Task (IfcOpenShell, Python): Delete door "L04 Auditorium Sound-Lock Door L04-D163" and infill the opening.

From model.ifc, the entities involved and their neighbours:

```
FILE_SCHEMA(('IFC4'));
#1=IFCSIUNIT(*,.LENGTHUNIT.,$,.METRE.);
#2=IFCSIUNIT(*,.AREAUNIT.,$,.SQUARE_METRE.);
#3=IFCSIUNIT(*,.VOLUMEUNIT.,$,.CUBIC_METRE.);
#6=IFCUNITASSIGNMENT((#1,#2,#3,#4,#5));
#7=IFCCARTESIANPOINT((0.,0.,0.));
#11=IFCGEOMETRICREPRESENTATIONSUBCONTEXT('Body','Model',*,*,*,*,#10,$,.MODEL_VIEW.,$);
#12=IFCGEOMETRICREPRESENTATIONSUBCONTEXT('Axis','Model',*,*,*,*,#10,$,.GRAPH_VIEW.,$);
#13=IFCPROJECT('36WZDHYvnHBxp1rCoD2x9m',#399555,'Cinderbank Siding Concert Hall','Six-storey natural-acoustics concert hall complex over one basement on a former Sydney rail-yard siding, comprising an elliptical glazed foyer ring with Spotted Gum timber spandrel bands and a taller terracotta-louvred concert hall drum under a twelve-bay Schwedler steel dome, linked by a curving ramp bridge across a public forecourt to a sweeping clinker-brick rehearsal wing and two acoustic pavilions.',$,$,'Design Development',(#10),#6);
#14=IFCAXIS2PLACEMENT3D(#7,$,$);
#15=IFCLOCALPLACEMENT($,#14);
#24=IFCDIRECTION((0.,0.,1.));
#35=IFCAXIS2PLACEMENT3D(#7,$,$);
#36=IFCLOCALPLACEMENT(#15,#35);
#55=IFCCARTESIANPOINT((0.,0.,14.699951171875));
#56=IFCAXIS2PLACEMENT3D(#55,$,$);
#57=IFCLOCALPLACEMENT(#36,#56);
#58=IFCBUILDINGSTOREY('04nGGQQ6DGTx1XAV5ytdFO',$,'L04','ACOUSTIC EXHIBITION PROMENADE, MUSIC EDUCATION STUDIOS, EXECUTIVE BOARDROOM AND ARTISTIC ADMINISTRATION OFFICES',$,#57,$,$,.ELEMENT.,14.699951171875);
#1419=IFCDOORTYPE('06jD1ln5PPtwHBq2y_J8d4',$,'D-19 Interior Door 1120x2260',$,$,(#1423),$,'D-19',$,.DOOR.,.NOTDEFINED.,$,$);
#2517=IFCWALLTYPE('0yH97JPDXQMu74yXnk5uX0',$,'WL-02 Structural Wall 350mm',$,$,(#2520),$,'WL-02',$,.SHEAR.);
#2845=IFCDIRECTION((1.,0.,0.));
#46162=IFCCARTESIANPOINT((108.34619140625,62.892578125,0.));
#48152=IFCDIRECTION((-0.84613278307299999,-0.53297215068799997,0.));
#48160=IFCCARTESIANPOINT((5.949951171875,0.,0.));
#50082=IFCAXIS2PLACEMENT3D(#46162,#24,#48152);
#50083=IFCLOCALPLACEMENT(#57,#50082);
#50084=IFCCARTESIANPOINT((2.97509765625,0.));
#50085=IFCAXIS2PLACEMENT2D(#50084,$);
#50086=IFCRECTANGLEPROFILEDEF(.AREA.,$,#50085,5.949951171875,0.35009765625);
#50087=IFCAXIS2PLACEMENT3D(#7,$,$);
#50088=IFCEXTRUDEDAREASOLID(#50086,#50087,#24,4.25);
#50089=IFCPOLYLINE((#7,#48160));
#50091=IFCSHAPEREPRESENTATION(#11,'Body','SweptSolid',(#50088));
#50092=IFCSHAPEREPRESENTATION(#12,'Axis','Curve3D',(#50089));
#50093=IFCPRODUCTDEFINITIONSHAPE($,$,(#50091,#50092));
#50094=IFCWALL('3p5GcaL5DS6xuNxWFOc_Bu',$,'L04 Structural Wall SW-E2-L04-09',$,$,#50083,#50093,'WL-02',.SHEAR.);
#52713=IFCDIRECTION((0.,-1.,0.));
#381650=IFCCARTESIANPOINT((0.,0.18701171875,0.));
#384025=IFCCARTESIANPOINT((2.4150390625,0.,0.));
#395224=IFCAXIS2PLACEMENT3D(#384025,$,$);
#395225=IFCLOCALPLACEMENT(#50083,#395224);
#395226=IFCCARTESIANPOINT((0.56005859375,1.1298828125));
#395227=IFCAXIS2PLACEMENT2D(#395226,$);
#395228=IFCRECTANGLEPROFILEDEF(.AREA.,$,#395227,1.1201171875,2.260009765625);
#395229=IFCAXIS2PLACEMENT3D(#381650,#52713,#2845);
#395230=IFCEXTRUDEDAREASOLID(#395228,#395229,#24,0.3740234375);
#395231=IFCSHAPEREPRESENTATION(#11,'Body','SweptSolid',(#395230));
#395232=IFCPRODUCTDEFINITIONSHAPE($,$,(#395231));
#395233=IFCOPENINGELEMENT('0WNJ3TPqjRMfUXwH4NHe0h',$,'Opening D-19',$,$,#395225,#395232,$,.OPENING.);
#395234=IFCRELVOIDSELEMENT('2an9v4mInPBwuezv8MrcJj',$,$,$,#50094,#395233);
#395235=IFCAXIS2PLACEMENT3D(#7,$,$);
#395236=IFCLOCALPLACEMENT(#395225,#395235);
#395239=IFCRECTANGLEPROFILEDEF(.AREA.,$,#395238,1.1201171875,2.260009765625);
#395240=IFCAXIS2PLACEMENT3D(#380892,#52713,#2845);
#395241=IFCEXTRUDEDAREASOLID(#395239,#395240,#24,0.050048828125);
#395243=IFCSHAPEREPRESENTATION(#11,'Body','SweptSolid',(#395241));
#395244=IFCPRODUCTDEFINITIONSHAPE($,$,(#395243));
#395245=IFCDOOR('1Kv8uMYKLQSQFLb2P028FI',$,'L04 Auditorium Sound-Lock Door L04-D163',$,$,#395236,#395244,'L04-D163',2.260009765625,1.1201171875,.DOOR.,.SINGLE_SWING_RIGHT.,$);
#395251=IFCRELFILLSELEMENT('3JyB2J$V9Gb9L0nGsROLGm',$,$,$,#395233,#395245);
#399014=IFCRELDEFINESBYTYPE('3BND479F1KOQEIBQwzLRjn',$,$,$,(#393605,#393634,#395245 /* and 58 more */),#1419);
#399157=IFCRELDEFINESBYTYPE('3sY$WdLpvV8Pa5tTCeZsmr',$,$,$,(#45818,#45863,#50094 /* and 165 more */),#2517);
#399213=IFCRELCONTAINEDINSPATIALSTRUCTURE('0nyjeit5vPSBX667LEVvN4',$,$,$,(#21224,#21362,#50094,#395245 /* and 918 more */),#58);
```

```python
import ifcopenshell
import ifcopenshell.api.feature
import ifcopenshell.api.root
import ifcopenshell.geom
import ifcopenshell.util.shape

model = ifcopenshell.open("model.ifc")
settings = ifcopenshell.geom.settings()


def volume(element):
    """Net volume in cubic metres, openings subtracted."""
    shape = ifcopenshell.geom.create_shape(settings, element)
    return ifcopenshell.util.shape.get_volume(shape.geometry)


door = model.by_guid("1Kv8uMYKLQSQFLb2P028FI")
opening = door.FillsVoids[0].RelatingOpeningElement
wall = opening.VoidsElements[0].RelatingBuildingElement
before = volume(wall)

ifcopenshell.api.root.remove_product(model, product=door)
ifcopenshell.api.feature.remove_feature(model, feature=opening)

after = volume(wall)

print(f"wall volume {before:.3f} -> {after:.3f} m3")

model.write("model_updated.ifc")
```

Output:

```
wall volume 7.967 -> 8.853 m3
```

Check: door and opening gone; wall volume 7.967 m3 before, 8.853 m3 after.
